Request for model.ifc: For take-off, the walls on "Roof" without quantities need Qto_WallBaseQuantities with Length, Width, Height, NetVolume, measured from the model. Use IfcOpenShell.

First a look at what the model holds.

```python
import ifcopenshell
import ifcopenshell.util.element
import ifcopenshell.util.unit

model = ifcopenshell.open("model.ifc")
print(model.schema)
for unit_type in ("LENGTHUNIT", "AREAUNIT", "VOLUMEUNIT"):
    print(unit_type, ifcopenshell.util.unit.calculate_unit_scale(model, unit_type))
storey = next(s for s in model.by_type("IfcBuildingStorey") if s.Name == "Roof")
walls = [e for e in ifcopenshell.util.element.get_decomposition(storey) if e.is_a("IfcWall")]
for e in sorted(walls, key=lambda e: e.id()):
    print(e.id(), e.is_a(), e.Name, list(ifcopenshell.util.element.get_psets(e, qtos_only=True)), sep=" | ")
```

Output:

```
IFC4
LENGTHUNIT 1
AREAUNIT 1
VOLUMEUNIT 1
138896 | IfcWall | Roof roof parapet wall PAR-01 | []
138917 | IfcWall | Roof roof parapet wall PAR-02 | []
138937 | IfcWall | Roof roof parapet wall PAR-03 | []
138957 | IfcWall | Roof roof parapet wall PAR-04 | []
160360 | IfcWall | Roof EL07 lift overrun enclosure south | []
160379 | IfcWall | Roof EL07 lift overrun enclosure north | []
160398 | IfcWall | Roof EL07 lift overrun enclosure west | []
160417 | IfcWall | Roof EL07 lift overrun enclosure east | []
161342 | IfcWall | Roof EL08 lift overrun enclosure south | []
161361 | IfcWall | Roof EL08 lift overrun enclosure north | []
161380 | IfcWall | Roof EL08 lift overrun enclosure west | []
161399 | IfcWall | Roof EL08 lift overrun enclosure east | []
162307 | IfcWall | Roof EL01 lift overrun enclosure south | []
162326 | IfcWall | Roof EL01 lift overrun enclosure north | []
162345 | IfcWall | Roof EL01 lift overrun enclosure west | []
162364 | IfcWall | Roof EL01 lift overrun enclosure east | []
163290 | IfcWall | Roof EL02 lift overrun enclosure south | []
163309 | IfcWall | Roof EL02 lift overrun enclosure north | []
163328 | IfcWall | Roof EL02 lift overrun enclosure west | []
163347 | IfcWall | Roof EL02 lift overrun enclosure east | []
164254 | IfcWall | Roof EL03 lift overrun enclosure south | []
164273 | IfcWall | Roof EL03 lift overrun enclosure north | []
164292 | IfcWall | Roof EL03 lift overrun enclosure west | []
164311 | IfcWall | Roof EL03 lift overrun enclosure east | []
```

```python
import ifcopenshell
import ifcopenshell.api.pset
import ifcopenshell.geom
import ifcopenshell.util.element
import ifcopenshell.util.shape
import ifcopenshell.util.unit

model = ifcopenshell.open("model.ifc")
unit_scale = ifcopenshell.util.unit.calculate_unit_scale(model)
volume_scale = ifcopenshell.util.unit.calculate_unit_scale(model, "VOLUMEUNIT")
settings = ifcopenshell.geom.settings()

storey = next(s for s in model.by_type("IfcBuildingStorey") if s.Name == "Roof")
walls = [e for e in ifcopenshell.util.element.get_decomposition(storey) if e.is_a("IfcWall")]

for e in sorted(walls, key=lambda e: e.id()):
    if ifcopenshell.util.element.get_psets(e, qtos_only=True, should_inherit=False):
        continue
    # Geometry comes back in metres, in the element's own axes.
    shape = ifcopenshell.geom.create_shape(settings, e)
    values = {
        "Length": ifcopenshell.util.shape.get_x(shape.geometry) / unit_scale,
        "Width": ifcopenshell.util.shape.get_y(shape.geometry) / unit_scale,
        "Height": ifcopenshell.util.shape.get_z(shape.geometry) / unit_scale,
        "NetVolume": ifcopenshell.util.shape.get_volume(shape.geometry) / volume_scale,
    }
    qto = ifcopenshell.api.pset.add_qto(model, product=e, name="Qto_WallBaseQuantities")
    ifcopenshell.api.pset.edit_qto(model, qto=qto, properties=values)
    print(e.id(), {k: round(v, 3) for k, v in values.items()})

model.write("model-out.ifc")
```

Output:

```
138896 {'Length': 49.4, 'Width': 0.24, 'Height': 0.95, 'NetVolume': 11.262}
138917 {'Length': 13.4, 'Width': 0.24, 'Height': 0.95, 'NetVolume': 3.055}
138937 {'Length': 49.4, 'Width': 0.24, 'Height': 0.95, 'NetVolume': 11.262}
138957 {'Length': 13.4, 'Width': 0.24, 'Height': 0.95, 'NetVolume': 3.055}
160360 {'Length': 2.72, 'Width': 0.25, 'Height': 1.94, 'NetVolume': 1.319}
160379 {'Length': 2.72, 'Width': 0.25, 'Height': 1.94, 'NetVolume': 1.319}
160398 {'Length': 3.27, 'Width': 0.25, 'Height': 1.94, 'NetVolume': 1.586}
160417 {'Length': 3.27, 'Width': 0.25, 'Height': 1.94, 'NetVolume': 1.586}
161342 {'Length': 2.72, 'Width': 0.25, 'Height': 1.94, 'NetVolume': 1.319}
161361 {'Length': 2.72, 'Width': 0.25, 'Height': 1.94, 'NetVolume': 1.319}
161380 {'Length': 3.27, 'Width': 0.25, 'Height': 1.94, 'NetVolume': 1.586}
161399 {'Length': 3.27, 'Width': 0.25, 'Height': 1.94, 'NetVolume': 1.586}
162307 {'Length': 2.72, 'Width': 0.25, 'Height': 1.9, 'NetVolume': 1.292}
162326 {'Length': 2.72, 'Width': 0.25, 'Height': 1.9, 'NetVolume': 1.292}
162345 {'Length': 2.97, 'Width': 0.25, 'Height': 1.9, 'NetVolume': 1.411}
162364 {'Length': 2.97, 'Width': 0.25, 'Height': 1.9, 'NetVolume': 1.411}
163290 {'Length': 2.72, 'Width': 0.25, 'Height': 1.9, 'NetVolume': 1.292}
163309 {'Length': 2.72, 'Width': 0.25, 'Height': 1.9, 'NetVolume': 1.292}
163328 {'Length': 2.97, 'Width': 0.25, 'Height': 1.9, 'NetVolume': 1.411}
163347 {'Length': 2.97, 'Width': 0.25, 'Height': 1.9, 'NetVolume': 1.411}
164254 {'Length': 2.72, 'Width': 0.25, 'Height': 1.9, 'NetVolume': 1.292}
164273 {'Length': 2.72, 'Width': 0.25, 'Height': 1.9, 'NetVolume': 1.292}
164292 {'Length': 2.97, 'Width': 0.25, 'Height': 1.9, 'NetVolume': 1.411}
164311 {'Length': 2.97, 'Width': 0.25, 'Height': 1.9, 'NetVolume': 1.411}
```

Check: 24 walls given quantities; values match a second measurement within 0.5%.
